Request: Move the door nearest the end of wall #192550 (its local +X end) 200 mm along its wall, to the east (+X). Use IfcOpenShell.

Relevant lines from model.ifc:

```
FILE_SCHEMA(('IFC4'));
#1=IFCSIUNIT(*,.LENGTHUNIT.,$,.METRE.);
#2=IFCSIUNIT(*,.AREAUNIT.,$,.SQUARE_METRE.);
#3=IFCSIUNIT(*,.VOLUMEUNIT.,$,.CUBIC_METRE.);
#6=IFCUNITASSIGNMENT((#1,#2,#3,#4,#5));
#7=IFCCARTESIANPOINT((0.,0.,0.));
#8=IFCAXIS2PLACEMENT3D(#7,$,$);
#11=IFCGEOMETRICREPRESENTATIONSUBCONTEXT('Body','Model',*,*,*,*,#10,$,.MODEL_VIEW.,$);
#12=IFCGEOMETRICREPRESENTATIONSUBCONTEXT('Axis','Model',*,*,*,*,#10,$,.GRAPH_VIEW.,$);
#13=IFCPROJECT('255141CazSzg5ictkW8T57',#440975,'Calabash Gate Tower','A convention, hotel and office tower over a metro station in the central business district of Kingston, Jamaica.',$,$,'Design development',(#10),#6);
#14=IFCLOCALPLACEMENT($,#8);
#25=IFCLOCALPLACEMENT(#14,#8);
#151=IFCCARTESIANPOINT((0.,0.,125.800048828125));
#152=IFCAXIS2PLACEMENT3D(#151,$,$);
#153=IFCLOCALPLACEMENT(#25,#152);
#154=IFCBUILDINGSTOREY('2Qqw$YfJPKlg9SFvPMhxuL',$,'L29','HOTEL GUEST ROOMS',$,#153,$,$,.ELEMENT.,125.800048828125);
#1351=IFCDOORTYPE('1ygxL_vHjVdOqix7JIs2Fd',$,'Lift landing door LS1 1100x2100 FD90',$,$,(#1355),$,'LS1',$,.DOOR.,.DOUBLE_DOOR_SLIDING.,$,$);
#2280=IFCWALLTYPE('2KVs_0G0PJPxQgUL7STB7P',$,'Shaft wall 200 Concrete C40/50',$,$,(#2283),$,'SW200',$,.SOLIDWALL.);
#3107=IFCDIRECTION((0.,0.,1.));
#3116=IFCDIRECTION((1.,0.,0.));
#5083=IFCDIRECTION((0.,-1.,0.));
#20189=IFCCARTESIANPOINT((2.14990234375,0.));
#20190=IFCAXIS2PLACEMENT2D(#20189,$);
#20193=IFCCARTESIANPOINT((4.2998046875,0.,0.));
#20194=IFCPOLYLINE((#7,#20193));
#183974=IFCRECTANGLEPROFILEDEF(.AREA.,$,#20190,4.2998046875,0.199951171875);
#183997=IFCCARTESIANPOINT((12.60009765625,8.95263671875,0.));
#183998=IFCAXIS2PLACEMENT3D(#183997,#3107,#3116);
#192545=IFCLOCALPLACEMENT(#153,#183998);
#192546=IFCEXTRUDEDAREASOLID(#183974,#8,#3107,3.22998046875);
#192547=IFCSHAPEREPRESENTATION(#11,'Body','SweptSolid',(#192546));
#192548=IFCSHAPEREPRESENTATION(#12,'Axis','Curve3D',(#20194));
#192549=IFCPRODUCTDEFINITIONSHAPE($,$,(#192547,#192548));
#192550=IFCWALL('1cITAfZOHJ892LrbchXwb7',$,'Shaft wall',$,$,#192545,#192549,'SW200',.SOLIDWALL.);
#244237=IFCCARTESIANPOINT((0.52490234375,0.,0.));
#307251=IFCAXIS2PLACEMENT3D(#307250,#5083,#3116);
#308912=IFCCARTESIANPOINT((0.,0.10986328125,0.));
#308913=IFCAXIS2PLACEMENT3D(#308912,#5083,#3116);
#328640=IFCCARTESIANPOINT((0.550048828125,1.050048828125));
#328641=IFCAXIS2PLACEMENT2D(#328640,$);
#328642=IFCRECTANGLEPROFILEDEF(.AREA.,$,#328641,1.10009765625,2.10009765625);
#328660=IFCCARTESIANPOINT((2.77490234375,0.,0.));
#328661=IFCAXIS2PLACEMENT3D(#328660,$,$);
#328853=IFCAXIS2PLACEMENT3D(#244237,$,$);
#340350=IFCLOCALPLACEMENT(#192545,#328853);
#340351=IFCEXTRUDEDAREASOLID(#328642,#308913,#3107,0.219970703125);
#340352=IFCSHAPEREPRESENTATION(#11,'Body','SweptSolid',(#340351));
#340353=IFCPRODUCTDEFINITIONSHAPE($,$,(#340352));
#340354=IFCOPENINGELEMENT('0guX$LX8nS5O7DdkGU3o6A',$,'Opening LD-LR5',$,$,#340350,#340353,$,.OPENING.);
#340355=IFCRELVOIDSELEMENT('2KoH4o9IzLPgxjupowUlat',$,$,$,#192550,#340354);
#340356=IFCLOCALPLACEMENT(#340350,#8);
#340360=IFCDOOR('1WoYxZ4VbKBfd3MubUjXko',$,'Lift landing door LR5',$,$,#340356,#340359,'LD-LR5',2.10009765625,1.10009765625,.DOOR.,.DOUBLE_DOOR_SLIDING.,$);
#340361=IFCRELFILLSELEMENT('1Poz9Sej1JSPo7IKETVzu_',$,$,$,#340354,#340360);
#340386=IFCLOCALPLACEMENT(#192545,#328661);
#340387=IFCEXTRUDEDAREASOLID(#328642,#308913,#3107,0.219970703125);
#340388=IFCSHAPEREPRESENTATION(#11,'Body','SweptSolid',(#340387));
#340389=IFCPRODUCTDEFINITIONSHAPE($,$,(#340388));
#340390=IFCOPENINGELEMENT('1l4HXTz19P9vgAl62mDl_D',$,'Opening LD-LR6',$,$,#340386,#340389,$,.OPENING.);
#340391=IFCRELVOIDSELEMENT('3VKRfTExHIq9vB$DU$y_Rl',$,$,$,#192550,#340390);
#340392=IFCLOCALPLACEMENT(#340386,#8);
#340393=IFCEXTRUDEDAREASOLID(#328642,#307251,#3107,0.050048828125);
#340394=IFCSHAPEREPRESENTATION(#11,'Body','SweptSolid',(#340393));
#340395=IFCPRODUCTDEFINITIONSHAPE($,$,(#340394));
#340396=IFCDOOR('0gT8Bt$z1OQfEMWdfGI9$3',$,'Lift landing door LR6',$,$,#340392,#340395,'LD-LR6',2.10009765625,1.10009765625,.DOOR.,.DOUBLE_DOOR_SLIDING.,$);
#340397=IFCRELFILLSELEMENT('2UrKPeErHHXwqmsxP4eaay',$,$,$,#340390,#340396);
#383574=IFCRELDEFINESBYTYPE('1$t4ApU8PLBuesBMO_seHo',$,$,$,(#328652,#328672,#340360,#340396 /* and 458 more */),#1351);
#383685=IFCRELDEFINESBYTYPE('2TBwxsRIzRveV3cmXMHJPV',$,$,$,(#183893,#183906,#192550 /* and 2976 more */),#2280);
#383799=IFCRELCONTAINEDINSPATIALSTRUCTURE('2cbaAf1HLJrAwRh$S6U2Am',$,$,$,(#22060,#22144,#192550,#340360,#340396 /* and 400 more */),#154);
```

```python
import ifcopenshell
import ifcopenshell.api.geometry
import ifcopenshell.util.placement

model = ifcopenshell.open("model.ifc")

door = model.by_guid("0gT8Bt$z1OQfEMWdfGI9$3")
opening = door.FillsVoids[0].RelatingOpeningElement
wall = opening.VoidsElements[0].RelatingBuildingElement

wall_matrix = ifcopenshell.util.placement.get_local_placement(wall.ObjectPlacement)
shift = wall_matrix[:3, 0] * 0.2
before = ifcopenshell.util.placement.get_local_placement(door.ObjectPlacement)[:3, 3].copy()

# The door is placed relative to its opening, so it follows when the opening moves.
matrix = ifcopenshell.util.placement.get_local_placement(opening.ObjectPlacement)
matrix[:3, 3] += shift
ifcopenshell.api.geometry.edit_object_placement(
    model, product=opening, matrix=matrix, is_si=False, should_transform_children=True
)

after = ifcopenshell.util.placement.get_local_placement(door.ObjectPlacement)[:3, 3]
print("door moved by", (after - before).round(3) + 0.0)

model.write("model_edited.ifc")
```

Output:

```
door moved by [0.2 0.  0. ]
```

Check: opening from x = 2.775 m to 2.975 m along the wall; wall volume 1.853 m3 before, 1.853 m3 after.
